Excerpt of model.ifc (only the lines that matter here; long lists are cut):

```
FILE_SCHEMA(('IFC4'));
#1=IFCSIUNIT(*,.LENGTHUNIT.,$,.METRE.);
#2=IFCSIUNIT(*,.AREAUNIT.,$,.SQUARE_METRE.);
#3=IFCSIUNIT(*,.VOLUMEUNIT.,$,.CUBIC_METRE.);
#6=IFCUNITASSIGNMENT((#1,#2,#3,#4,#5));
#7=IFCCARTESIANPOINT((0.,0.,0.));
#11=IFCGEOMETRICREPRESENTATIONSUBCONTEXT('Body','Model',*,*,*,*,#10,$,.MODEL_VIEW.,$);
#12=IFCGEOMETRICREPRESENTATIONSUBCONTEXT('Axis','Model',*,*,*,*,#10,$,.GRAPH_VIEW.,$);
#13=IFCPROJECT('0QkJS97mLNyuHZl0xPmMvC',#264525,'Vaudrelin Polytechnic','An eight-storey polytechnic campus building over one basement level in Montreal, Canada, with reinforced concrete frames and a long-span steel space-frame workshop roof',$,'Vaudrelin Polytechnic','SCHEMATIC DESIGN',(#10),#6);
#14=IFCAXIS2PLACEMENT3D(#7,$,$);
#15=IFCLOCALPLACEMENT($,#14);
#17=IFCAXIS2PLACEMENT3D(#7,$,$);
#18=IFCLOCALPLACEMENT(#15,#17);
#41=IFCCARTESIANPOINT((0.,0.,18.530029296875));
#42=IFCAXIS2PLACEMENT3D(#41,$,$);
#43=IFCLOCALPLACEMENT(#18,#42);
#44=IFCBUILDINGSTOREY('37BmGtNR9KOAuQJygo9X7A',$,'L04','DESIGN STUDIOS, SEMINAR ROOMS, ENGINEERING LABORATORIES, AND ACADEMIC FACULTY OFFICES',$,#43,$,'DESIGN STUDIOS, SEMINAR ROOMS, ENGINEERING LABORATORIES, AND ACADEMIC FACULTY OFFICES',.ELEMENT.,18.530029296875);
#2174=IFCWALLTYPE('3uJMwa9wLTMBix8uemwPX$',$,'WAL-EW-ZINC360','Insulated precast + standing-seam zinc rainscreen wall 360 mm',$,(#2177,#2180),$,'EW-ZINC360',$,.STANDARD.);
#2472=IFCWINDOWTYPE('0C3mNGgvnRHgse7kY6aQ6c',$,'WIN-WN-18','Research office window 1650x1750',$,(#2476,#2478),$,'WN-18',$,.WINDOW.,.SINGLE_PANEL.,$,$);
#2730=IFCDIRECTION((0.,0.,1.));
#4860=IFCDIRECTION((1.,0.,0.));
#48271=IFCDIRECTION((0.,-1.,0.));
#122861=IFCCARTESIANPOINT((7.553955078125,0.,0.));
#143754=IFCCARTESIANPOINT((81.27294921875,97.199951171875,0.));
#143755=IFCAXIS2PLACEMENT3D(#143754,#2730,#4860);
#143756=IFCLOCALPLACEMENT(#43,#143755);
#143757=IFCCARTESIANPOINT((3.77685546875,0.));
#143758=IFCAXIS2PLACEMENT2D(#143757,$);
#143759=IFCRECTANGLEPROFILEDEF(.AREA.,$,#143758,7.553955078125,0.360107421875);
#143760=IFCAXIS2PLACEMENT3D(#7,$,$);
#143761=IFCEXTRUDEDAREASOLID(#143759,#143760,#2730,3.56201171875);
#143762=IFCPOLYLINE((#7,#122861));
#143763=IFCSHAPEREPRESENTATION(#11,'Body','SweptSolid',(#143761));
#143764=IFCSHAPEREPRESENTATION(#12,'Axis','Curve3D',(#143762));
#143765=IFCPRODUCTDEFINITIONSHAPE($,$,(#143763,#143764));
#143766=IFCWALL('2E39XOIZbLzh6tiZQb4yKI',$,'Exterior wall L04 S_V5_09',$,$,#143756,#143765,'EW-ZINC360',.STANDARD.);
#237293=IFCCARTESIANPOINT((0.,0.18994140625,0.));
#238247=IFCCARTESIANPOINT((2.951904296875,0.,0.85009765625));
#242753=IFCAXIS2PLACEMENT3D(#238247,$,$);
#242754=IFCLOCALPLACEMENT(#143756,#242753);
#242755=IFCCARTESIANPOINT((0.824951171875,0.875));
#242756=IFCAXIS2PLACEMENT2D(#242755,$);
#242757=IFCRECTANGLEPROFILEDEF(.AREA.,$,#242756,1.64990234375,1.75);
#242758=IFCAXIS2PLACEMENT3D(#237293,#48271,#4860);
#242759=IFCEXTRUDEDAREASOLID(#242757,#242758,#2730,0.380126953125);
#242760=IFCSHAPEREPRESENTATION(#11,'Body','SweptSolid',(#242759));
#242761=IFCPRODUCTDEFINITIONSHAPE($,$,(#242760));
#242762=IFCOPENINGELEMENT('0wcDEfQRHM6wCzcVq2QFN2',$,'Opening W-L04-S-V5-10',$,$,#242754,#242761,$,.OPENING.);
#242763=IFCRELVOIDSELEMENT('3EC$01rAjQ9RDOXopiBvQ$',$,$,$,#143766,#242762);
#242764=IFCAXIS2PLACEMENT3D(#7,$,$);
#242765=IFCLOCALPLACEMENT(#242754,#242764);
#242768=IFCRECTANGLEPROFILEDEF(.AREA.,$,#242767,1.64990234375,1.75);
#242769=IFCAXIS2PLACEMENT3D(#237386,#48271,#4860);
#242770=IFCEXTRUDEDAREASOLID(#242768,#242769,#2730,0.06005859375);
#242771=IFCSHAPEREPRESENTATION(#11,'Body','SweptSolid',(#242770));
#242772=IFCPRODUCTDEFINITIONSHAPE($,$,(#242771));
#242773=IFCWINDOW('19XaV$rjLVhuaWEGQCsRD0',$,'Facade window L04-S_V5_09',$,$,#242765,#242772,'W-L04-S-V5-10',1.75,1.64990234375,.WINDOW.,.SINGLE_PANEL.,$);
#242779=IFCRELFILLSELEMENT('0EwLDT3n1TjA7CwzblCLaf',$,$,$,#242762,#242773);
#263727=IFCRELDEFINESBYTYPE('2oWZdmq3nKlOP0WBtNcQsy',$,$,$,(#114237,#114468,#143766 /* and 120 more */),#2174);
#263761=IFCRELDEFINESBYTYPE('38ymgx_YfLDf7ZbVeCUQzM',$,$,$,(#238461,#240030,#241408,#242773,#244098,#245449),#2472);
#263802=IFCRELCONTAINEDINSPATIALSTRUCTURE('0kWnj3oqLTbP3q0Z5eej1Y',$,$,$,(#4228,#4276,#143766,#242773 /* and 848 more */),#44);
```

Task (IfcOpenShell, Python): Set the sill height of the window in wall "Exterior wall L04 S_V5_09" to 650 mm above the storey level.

```python
import numpy as np
import ifcopenshell
import ifcopenshell.api.geometry
import ifcopenshell.geom
import ifcopenshell.util.element
import ifcopenshell.util.placement
import ifcopenshell.util.shape
import ifcopenshell.util.unit

model = ifcopenshell.open("model.ifc")
unit_scale = ifcopenshell.util.unit.calculate_unit_scale(model)

window = model.by_guid("19XaV$rjLVhuaWEGQCsRD0")
opening = window.FillsVoids[0].RelatingOpeningElement
storey = ifcopenshell.util.element.get_container(window, ifc_class="IfcBuildingStorey")
level = ifcopenshell.util.placement.get_local_placement(storey.ObjectPlacement)[2, 3]

# The opening's origin need not be at the sill, so measure its lowest point.
shape = ifcopenshell.geom.create_shape(ifcopenshell.geom.settings(), opening)
bottom = ifcopenshell.util.shape.get_shape_bottom_elevation(shape, shape.geometry) / unit_scale
dz = level + 0.65 - bottom

shift = np.array([0.0, 0.0, dz])
# The window is placed relative to its opening, so it follows when the opening moves.
matrix = ifcopenshell.util.placement.get_local_placement(opening.ObjectPlacement)
matrix[:3, 3] += shift
ifcopenshell.api.geometry.edit_object_placement(
    model, product=opening, matrix=matrix, is_si=False, should_transform_children=True
)

print(f"moved by {dz * unit_scale:+.3f} m")

model.write("model_edited.ifc")
```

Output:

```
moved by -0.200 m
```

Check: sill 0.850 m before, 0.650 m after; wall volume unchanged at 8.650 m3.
